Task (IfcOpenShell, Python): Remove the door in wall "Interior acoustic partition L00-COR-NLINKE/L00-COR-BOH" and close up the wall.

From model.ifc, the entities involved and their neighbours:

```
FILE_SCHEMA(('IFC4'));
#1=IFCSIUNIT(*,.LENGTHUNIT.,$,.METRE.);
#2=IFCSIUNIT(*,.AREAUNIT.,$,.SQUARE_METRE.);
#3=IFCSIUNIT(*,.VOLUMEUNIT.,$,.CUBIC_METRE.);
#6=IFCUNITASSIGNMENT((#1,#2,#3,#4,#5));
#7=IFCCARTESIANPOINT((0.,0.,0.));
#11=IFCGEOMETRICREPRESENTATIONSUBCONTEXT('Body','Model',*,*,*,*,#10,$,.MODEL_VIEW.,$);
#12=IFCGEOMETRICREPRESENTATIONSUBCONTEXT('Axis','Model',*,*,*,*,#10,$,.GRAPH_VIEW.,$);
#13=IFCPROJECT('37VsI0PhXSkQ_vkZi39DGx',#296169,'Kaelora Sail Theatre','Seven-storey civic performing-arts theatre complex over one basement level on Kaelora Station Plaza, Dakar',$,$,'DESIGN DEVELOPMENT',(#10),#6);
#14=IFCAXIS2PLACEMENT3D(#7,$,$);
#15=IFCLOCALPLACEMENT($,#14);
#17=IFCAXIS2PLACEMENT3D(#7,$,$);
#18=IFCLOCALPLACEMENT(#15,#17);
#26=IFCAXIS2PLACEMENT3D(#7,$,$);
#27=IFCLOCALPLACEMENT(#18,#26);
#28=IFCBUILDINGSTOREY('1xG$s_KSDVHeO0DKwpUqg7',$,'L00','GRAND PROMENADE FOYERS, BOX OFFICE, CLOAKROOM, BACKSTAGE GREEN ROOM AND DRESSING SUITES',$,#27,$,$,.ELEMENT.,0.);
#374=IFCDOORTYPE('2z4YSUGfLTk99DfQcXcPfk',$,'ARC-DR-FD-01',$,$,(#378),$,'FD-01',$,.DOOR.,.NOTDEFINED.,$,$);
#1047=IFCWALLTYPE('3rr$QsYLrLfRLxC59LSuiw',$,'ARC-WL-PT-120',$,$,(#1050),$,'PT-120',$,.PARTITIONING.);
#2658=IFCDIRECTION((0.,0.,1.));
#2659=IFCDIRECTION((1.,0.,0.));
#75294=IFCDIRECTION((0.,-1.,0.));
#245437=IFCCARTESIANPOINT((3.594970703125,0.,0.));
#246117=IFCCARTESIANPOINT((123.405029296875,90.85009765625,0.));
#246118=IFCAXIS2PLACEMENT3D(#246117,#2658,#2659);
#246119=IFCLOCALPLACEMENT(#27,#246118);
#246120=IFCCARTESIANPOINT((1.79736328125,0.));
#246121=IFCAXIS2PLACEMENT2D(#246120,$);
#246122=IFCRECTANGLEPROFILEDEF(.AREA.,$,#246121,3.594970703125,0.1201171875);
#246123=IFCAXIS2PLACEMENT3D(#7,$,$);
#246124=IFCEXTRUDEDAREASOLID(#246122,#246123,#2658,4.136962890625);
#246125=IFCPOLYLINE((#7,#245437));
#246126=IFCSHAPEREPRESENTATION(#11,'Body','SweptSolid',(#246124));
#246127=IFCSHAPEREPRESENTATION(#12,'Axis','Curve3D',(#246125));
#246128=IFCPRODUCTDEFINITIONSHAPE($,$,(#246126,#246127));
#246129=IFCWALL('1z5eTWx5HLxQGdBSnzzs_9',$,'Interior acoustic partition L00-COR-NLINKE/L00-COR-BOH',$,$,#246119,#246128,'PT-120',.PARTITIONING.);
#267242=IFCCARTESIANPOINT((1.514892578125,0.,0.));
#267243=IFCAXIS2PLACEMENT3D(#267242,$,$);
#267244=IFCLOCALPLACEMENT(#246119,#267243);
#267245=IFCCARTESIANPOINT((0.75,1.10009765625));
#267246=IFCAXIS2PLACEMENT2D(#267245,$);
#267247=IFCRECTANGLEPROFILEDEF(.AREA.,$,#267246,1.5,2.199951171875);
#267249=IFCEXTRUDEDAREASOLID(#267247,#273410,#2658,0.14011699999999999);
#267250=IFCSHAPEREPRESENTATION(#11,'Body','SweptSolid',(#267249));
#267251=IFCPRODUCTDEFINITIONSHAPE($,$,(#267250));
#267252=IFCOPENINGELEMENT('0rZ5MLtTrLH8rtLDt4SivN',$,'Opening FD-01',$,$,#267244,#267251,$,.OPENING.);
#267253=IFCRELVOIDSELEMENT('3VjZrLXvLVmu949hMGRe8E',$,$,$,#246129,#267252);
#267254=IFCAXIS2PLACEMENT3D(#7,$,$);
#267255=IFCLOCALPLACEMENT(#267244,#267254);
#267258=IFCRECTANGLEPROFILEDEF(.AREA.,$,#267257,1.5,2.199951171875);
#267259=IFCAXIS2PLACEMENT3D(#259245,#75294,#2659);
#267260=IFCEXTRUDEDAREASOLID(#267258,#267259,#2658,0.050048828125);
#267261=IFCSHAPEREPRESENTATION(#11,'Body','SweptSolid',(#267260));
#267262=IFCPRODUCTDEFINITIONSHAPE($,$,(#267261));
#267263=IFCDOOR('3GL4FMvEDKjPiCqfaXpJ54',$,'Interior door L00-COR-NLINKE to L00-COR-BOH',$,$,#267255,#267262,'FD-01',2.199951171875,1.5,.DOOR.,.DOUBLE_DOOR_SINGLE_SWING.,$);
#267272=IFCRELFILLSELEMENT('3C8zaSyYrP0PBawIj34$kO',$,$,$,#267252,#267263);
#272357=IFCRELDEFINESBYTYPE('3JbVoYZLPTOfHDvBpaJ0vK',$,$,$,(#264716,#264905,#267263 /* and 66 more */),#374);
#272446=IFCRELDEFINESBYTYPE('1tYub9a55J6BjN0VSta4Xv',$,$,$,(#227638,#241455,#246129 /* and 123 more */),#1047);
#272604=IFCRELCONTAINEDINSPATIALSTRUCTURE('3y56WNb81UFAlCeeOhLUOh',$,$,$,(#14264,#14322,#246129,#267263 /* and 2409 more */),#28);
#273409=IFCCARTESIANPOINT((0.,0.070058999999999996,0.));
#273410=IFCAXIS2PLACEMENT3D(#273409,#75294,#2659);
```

```python
import ifcopenshell
import ifcopenshell.api.feature
import ifcopenshell.api.root
import ifcopenshell.geom
import ifcopenshell.util.shape

model = ifcopenshell.open("model.ifc")
settings = ifcopenshell.geom.settings()


def volume(element):
    """Net volume in cubic metres, openings subtracted."""
    shape = ifcopenshell.geom.create_shape(settings, element)
    return ifcopenshell.util.shape.get_volume(shape.geometry)


door = model.by_guid("3GL4FMvEDKjPiCqfaXpJ54")
opening = door.FillsVoids[0].RelatingOpeningElement
wall = opening.VoidsElements[0].RelatingBuildingElement
before = volume(wall)

ifcopenshell.api.root.remove_product(model, product=door)
ifcopenshell.api.feature.remove_feature(model, feature=opening)

after = volume(wall)

print(f"wall volume {before:.3f} -> {after:.3f} m3")

model.write("model_rev.ifc")
```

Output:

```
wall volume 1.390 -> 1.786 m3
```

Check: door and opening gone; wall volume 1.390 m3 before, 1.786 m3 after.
